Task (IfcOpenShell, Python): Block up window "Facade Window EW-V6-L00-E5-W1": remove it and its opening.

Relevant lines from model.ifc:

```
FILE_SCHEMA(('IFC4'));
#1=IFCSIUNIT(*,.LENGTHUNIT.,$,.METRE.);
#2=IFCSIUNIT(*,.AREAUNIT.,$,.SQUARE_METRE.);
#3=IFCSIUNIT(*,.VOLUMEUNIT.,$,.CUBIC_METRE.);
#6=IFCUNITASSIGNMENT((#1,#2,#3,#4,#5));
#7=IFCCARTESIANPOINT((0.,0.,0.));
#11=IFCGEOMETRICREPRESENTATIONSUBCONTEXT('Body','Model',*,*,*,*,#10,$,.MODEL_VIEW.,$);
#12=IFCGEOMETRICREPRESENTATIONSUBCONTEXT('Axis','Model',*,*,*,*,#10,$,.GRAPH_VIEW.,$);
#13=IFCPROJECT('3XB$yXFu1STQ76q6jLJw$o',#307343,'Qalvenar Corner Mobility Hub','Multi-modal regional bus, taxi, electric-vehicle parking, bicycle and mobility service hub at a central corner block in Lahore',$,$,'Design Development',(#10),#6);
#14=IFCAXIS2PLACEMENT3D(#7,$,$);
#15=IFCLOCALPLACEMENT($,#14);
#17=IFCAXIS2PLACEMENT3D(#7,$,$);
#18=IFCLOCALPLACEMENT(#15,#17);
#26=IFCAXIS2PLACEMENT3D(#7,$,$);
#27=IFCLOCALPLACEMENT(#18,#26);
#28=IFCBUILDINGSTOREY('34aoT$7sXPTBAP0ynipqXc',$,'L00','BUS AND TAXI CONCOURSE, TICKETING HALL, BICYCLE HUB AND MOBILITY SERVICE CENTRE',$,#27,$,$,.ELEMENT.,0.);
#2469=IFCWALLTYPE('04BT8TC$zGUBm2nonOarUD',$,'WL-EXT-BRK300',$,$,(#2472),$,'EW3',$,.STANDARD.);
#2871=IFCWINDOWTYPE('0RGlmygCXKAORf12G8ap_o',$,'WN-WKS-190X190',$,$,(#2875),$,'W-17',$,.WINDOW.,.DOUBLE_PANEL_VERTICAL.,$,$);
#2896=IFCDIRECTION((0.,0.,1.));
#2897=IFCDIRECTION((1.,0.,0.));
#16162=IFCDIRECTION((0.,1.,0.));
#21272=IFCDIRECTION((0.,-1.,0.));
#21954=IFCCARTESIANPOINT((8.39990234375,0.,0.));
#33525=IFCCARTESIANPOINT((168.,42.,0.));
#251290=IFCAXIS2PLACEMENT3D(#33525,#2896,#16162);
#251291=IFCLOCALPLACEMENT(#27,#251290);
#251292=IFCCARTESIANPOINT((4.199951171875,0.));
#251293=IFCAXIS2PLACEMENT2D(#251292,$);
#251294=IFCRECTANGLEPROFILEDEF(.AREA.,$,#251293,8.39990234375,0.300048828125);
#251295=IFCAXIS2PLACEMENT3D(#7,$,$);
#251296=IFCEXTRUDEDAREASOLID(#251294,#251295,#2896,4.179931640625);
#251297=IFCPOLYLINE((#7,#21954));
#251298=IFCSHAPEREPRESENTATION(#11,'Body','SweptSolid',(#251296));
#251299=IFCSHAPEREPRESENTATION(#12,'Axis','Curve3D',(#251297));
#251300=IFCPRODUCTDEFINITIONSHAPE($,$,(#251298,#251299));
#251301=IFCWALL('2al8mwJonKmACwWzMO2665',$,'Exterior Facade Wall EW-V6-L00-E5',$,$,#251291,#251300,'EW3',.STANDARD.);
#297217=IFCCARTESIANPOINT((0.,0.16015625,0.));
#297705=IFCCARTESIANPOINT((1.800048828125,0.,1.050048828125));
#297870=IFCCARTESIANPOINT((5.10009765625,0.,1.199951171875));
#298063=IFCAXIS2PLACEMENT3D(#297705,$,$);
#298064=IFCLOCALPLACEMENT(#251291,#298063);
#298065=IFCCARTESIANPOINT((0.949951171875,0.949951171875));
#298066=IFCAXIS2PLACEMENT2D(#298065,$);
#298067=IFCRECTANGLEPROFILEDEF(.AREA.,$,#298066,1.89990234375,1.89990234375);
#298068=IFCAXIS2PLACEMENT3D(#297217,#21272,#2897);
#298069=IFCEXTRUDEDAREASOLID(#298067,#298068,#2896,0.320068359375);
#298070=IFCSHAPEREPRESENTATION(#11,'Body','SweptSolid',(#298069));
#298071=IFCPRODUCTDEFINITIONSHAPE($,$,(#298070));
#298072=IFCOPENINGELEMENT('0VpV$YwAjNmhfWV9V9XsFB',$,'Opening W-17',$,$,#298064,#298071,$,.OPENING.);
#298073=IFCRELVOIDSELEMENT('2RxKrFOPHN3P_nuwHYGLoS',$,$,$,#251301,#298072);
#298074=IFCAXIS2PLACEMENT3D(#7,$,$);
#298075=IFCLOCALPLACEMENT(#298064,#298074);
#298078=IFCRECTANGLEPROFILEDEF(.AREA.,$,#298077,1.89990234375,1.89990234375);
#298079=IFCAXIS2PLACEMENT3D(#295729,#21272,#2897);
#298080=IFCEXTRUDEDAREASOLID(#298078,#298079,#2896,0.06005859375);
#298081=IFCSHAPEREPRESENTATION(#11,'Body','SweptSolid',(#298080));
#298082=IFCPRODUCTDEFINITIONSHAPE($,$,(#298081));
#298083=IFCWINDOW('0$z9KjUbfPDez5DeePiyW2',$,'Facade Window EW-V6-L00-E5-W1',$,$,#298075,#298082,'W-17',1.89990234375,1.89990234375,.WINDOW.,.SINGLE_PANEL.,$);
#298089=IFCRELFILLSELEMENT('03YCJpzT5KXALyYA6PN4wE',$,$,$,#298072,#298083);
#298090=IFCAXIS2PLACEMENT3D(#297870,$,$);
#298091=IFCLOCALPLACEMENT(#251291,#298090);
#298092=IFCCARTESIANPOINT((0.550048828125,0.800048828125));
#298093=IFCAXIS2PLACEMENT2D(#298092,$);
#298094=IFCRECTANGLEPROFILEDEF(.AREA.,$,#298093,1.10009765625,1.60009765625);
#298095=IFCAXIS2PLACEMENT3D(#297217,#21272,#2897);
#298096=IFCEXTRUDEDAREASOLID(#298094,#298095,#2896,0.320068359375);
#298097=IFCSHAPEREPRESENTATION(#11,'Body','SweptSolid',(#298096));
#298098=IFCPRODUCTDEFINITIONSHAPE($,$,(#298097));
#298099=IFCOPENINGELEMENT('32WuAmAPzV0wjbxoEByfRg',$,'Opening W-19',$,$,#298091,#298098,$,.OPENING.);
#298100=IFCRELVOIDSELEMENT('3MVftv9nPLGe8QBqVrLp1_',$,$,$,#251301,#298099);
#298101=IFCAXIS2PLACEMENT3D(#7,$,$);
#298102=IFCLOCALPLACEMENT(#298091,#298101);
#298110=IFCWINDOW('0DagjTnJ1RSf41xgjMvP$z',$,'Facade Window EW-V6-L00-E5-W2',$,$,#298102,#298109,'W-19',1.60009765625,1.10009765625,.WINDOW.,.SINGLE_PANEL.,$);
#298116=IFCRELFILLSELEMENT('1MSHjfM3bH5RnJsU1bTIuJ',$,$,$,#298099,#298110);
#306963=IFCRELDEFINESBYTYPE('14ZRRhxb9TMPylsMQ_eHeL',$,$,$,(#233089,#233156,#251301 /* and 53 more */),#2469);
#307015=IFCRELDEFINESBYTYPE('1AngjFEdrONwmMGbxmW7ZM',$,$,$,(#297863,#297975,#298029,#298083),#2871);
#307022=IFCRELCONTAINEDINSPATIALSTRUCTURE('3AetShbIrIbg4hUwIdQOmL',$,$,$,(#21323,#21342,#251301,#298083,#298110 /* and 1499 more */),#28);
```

```python
import ifcopenshell
import ifcopenshell.api.feature
import ifcopenshell.api.root
import ifcopenshell.geom
import ifcopenshell.util.shape

model = ifcopenshell.open("model.ifc")
settings = ifcopenshell.geom.settings()


def volume(element):
    """Net volume in cubic metres, openings subtracted."""
    shape = ifcopenshell.geom.create_shape(settings, element)
    return ifcopenshell.util.shape.get_volume(shape.geometry)


window = model.by_guid("0$z9KjUbfPDez5DeePiyW2")
opening = window.FillsVoids[0].RelatingOpeningElement
wall = opening.VoidsElements[0].RelatingBuildingElement
before = volume(wall)

ifcopenshell.api.root.remove_product(model, product=window)
ifcopenshell.api.feature.remove_feature(model, feature=opening)

after = volume(wall)

print(f"wall volume {before:.3f} -> {after:.3f} m3")

model.write("model_rev.ifc")
```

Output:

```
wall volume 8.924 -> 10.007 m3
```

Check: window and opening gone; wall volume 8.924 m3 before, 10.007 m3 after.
